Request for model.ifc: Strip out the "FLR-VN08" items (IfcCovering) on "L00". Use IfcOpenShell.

First a look at what the model holds.

```python
import ifcopenshell
import ifcopenshell.util.element

model = ifcopenshell.open("model.ifc")
print(model.schema)
storey = next(s for s in model.by_type("IfcBuildingStorey") if s.Name == "L00")
coverings = [e for e in ifcopenshell.util.element.get_decomposition(storey) if e.is_a("IfcCovering")]
seen = {}
for e in coverings:
    element_type = ifcopenshell.util.element.get_type(e)
    name = element_type.Name if element_type not in (None, e) else None
    seen[name] = seen.get(name, 0) + 1
for name, count in sorted(seen.items(), key=str):
    print(count, "x", name)
```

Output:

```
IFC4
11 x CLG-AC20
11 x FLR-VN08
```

```python
import ifcopenshell
import ifcopenshell.api.root
import ifcopenshell.util.element

model = ifcopenshell.open("model.ifc")

storey = next(s for s in model.by_type("IfcBuildingStorey") if s.Name == "L00")
coverings = [e for e in ifcopenshell.util.element.get_decomposition(storey) if e.is_a("IfcCovering")]
targets = [e for e in coverings if (t := ifcopenshell.util.element.get_type(e)) not in (None, e) and t.Name == "FLR-VN08"]

for e in targets:
    ifcopenshell.api.root.remove_product(model, product=e)
print(len(targets), "removed")

model.write("model-out.ifc")
```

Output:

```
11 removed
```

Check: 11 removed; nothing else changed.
